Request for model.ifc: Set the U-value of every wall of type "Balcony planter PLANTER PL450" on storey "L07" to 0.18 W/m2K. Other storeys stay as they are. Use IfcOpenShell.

First a look at what the model holds.

```python
import ifcopenshell
import ifcopenshell.util.element

model = ifcopenshell.open("model.ifc")
print(model.schema)
storey = next(s for s in model.by_type("IfcBuildingStorey") if s.Name == "L07")
walls = [e for e in ifcopenshell.util.element.get_decomposition(storey) if e.is_a("IfcWall")]
seen = {}
for e in walls:
    element_type = ifcopenshell.util.element.get_type(e)
    key = (element_type.Name if element_type != e and element_type else None, ifcopenshell.util.element.get_pset(e, "Pset_WallCommon", "ThermalTransmittance"))
    seen[key] = seen.get(key, 0) + 1
for (name, value), count in sorted(seen.items(), key=str):
    print(count, "x", name, "|", value)
```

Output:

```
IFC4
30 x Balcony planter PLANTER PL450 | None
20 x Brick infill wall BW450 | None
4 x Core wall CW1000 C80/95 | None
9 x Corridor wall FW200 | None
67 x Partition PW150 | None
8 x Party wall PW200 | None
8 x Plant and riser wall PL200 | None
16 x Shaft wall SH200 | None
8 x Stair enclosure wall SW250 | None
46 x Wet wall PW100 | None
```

```python
import ifcopenshell
import ifcopenshell.api.pset
import ifcopenshell.util.element

model = ifcopenshell.open("model.ifc")

storey = next(s for s in model.by_type("IfcBuildingStorey") if s.Name == "L07")
walls = [e for e in ifcopenshell.util.element.get_decomposition(storey) if e.is_a("IfcWall")]

count = 0
for e in walls:
    element_type = ifcopenshell.util.element.get_type(e)
    if element_type in (None, e) or element_type.Name != "Balcony planter PLANTER PL450":
        continue
    found = ifcopenshell.util.element.get_pset(e, "Pset_WallCommon", should_inherit=False)
    if found:
        pset = model.by_id(found["id"])
        if len(ifcopenshell.util.element.get_elements_by_pset(pset)) > 1:
            pset = ifcopenshell.api.pset.unshare_pset(model, products=[e], pset=pset)[0]
    else:
        pset = ifcopenshell.api.pset.add_pset(model, product=e, name="Pset_WallCommon")
    ifcopenshell.api.pset.edit_pset(model, pset=pset, properties={"ThermalTransmittance": 0.18})
    count += 1

print(count, "walls updated")

model.write("model_updated.ifc")
```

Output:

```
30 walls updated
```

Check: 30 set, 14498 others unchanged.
